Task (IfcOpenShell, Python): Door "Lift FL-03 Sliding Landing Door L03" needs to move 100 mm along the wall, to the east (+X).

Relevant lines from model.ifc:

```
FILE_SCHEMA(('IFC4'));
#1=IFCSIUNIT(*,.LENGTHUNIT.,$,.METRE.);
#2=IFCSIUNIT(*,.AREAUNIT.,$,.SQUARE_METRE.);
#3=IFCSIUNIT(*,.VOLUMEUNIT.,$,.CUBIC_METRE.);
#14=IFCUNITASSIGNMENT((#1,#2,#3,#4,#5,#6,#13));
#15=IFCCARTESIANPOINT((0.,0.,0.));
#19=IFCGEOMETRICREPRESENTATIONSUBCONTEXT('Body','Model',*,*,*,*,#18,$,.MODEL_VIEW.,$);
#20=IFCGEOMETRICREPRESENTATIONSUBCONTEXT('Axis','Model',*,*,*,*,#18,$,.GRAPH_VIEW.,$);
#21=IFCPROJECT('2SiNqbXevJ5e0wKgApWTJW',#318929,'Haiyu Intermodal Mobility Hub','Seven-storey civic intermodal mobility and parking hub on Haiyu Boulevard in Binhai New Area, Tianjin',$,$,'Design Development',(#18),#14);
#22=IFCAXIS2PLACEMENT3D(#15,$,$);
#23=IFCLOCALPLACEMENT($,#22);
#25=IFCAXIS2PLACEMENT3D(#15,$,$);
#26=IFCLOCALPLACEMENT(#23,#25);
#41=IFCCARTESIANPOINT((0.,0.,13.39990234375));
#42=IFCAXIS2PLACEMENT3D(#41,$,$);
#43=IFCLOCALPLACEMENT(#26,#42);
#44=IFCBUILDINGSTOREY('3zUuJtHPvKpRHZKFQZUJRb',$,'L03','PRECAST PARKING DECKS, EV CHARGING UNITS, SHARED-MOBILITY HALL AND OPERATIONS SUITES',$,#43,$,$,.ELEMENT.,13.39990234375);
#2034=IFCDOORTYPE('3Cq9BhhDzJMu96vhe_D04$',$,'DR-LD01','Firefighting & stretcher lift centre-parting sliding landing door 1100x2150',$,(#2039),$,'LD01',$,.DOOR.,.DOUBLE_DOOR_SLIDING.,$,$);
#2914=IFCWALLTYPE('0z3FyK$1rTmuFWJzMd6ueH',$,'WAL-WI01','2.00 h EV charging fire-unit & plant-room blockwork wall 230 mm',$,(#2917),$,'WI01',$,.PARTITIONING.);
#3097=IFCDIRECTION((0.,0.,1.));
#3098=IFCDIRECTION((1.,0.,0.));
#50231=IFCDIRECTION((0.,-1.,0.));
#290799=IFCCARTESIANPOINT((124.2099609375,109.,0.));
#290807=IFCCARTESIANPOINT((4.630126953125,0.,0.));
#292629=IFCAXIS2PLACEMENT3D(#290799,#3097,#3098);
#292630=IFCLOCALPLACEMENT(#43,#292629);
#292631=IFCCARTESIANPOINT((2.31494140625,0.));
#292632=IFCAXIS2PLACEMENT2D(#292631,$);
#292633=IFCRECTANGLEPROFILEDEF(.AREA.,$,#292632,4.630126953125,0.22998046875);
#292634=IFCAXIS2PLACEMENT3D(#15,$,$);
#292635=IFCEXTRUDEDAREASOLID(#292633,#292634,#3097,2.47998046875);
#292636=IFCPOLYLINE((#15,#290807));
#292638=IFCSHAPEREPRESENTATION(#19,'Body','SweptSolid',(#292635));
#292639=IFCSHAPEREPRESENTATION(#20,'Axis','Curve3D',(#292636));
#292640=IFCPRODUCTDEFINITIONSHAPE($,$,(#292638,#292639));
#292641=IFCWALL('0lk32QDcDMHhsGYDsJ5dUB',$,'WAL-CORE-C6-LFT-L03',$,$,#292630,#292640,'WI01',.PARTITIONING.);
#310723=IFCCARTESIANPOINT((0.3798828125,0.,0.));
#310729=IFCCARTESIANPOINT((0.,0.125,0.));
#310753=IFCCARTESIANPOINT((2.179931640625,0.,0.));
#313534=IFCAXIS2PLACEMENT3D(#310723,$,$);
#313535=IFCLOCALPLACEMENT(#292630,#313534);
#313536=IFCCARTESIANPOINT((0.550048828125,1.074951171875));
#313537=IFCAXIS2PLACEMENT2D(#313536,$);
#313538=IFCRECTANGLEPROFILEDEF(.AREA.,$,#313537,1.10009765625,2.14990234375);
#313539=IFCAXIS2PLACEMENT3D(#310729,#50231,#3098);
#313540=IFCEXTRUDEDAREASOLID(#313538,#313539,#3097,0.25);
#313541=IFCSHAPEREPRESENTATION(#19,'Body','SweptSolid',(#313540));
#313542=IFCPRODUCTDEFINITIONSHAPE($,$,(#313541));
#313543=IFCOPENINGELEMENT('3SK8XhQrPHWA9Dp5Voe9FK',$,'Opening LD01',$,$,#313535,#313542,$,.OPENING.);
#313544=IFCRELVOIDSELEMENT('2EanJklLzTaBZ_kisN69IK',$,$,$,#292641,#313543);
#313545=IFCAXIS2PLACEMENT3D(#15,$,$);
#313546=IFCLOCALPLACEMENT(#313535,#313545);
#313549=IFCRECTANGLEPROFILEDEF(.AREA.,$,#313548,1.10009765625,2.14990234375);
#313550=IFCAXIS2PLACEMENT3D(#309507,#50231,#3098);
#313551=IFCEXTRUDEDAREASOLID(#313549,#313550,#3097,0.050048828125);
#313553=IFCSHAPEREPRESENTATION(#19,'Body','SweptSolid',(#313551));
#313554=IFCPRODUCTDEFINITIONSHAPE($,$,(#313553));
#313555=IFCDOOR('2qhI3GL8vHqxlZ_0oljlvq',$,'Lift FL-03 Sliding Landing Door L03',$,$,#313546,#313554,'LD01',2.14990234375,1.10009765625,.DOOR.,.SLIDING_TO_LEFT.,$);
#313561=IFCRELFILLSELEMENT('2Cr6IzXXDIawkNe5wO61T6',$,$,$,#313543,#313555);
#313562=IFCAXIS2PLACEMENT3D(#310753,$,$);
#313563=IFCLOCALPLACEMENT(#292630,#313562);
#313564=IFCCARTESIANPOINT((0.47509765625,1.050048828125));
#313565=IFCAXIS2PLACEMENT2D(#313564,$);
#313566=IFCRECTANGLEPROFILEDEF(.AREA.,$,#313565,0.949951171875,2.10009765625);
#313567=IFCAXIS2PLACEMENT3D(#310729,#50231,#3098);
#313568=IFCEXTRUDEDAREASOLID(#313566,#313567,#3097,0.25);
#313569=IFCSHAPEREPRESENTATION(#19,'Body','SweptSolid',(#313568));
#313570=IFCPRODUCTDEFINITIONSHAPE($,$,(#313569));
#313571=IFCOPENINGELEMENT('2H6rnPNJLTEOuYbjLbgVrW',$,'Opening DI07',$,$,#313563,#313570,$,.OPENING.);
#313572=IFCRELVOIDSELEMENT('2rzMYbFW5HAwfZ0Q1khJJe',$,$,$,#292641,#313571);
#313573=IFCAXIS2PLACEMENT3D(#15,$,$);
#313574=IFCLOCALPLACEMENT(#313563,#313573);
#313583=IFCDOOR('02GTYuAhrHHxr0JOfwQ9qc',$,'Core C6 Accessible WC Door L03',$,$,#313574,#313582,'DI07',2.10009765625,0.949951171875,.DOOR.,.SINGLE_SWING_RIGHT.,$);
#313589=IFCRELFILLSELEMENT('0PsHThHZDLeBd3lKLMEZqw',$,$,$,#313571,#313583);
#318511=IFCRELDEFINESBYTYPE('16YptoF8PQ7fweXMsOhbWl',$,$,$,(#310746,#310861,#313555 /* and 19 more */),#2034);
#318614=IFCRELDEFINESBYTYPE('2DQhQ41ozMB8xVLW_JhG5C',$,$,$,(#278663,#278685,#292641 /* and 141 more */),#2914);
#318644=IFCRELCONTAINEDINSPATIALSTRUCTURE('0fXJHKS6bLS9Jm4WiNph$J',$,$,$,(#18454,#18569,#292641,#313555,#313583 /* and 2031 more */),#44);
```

```python
import ifcopenshell
import ifcopenshell.api.geometry
import ifcopenshell.util.placement
import ifcopenshell.util.unit

model = ifcopenshell.open("model.ifc")
unit_scale = ifcopenshell.util.unit.calculate_unit_scale(model)

door = model.by_guid("2qhI3GL8vHqxlZ_0oljlvq")
opening = door.FillsVoids[0].RelatingOpeningElement
wall = opening.VoidsElements[0].RelatingBuildingElement

wall_matrix = ifcopenshell.util.placement.get_local_placement(wall.ObjectPlacement)
shift = wall_matrix[:3, 0] * 0.1 / unit_scale
before = ifcopenshell.util.placement.get_local_placement(door.ObjectPlacement)[:3, 3].copy()

# The door is placed relative to its opening, so it follows when the opening moves.
matrix = ifcopenshell.util.placement.get_local_placement(opening.ObjectPlacement)
matrix[:3, 3] += shift
ifcopenshell.api.geometry.edit_object_placement(
    model, product=opening, matrix=matrix, is_si=False, should_transform_children=True
)

after = ifcopenshell.util.placement.get_local_placement(door.ObjectPlacement)[:3, 3]
print("door moved by", (after - before).round(3) + 0.0)

model.write("model_v2.ifc")
```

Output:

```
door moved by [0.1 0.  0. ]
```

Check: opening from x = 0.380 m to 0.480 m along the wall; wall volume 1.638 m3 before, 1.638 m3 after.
